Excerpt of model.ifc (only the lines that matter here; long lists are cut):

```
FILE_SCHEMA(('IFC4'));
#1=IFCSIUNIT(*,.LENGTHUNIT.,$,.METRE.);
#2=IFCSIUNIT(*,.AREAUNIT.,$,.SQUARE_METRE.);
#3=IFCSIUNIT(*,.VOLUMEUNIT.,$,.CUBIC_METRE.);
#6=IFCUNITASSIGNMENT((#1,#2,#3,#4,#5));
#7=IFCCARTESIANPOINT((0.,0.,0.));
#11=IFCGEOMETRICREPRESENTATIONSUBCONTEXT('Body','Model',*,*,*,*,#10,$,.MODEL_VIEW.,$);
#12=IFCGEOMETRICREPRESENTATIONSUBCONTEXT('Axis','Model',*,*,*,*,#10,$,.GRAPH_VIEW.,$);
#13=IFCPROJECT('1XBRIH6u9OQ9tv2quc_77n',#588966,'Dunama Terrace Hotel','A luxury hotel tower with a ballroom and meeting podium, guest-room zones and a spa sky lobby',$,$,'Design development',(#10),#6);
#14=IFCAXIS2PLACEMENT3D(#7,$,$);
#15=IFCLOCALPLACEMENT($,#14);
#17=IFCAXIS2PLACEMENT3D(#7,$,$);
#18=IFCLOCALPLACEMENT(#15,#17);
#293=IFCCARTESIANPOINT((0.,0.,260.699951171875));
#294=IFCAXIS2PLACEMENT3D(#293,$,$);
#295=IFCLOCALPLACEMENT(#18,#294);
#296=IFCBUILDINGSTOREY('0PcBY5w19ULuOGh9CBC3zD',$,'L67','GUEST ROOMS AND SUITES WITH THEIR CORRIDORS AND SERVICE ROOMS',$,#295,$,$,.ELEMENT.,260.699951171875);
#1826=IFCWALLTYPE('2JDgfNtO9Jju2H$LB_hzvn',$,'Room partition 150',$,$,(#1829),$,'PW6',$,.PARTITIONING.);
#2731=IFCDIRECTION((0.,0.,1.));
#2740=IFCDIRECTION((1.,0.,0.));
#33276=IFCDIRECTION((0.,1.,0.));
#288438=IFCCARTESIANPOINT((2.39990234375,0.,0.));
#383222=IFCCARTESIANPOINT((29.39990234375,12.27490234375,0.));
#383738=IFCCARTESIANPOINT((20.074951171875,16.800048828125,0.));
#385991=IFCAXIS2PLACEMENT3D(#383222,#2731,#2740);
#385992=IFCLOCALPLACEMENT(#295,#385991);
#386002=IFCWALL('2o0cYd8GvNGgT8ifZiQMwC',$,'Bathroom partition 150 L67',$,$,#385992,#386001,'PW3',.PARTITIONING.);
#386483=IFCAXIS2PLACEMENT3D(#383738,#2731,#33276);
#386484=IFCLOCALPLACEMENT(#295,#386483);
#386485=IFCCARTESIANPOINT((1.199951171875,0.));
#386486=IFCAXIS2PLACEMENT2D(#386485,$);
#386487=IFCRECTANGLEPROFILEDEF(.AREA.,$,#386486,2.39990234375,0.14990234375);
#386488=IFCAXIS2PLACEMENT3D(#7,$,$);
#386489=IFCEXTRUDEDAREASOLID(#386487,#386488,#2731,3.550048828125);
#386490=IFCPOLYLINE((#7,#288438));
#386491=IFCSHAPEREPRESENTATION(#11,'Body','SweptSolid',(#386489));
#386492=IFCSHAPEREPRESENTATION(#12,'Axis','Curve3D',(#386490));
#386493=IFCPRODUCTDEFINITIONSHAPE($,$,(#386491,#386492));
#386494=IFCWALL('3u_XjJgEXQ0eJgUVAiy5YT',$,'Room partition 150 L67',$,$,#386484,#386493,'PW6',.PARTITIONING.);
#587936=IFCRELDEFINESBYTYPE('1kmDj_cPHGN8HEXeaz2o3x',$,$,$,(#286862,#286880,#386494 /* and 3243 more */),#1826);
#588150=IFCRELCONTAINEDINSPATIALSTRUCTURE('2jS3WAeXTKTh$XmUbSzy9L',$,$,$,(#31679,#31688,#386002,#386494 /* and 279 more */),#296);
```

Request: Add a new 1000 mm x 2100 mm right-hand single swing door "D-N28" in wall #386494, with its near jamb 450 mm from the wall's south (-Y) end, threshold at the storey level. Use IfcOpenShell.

```python
import numpy as np
import ifcopenshell
import ifcopenshell.api.feature
import ifcopenshell.api.geometry
import ifcopenshell.api.root
import ifcopenshell.api.spatial
import ifcopenshell.geom
import ifcopenshell.util.element
import ifcopenshell.util.placement
import ifcopenshell.util.representation
import ifcopenshell.util.shape
import ifcopenshell.util.unit

model = ifcopenshell.open("model.ifc")
unit_scale = ifcopenshell.util.unit.calculate_unit_scale(model)
settings = ifcopenshell.geom.settings()


def volume(element):
    """Net volume in cubic metres, openings subtracted."""
    shape = ifcopenshell.geom.create_shape(settings, element)
    return ifcopenshell.util.shape.get_volume(shape.geometry)


wall = model.by_guid("3u_XjJgEXQ0eJgUVAiy5YT")
storey = ifcopenshell.util.element.get_container(wall, ifc_class="IfcBuildingStorey")
context = ifcopenshell.util.representation.get_context(model, "Model", "Body", "MODEL_VIEW")
before = volume(wall)

width, height, from_end, sill = 1, 2.1, 0.45, 0.0  # metres

# The wall runs along its own X axis, and the end named is its -X end.
wall_shape = ifcopenshell.geom.create_shape(settings, wall)
x, y, z = ifcopenshell.util.shape.get_vertices(wall_shape.geometry).T
start = x.min() + from_end
face, thickness = float(y.min()), float(y.max() - y.min())
wall_matrix = ifcopenshell.util.placement.get_local_placement(wall.ObjectPlacement)
level = ifcopenshell.util.placement.get_local_placement(storey.ObjectPlacement)[2, 3]


def in_wall(x, y):
    """Placement at x, y metres in the wall's axes, at sill height."""
    matrix = wall_matrix.copy()
    matrix[:, 3] = wall_matrix @ np.array([x / unit_scale, y / unit_scale, 0.0, 1.0])
    matrix[2, 3] = level + sill / unit_scale
    return matrix


# Opening: a box that overshoots both wall faces by 50 mm.
opening = ifcopenshell.api.root.create_entity(model, ifc_class="IfcOpeningElement", predefined_type="OPENING")
box = ifcopenshell.api.geometry.add_wall_representation(
    model, context=context, length=width, height=height, thickness=thickness + 0.1
)
ifcopenshell.api.geometry.assign_representation(model, product=opening, representation=box)
ifcopenshell.api.geometry.edit_object_placement(model, product=opening, matrix=in_wall(start, face - 0.05), is_si=False)
ifcopenshell.api.feature.add_feature(model, feature=opening, element=wall)

door = ifcopenshell.api.root.create_entity(model, ifc_class="IfcDoor", name="D-N28", predefined_type="DOOR")
door.OverallWidth, door.OverallHeight = width / unit_scale, height / unit_scale
door.OperationType = "SINGLE_SWING_RIGHT"
body = ifcopenshell.api.geometry.add_door_representation(
    model,
    context=context,
    overall_width=door.OverallWidth,
    overall_height=door.OverallHeight,
    operation_type="SINGLE_SWING_RIGHT",
    lining_properties={"LiningDepth": thickness / unit_scale, "ThresholdDepth": thickness / unit_scale},
)
ifcopenshell.api.geometry.assign_representation(model, product=door, representation=body)
ifcopenshell.api.spatial.assign_container(model, products=[door], relating_structure=storey)
ifcopenshell.api.feature.add_filling(model, opening=opening, element=door)

# The lining spans the wall, so the door starts at the wall face.
ifcopenshell.api.geometry.edit_object_placement(model, product=door, matrix=in_wall(start, face), is_si=False)

after = volume(wall)

print(f"wall volume {before:.3f} -> {after:.3f} m3")

model.write("model_edited.ifc")
```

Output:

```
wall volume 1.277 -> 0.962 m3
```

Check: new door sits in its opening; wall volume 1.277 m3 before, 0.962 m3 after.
